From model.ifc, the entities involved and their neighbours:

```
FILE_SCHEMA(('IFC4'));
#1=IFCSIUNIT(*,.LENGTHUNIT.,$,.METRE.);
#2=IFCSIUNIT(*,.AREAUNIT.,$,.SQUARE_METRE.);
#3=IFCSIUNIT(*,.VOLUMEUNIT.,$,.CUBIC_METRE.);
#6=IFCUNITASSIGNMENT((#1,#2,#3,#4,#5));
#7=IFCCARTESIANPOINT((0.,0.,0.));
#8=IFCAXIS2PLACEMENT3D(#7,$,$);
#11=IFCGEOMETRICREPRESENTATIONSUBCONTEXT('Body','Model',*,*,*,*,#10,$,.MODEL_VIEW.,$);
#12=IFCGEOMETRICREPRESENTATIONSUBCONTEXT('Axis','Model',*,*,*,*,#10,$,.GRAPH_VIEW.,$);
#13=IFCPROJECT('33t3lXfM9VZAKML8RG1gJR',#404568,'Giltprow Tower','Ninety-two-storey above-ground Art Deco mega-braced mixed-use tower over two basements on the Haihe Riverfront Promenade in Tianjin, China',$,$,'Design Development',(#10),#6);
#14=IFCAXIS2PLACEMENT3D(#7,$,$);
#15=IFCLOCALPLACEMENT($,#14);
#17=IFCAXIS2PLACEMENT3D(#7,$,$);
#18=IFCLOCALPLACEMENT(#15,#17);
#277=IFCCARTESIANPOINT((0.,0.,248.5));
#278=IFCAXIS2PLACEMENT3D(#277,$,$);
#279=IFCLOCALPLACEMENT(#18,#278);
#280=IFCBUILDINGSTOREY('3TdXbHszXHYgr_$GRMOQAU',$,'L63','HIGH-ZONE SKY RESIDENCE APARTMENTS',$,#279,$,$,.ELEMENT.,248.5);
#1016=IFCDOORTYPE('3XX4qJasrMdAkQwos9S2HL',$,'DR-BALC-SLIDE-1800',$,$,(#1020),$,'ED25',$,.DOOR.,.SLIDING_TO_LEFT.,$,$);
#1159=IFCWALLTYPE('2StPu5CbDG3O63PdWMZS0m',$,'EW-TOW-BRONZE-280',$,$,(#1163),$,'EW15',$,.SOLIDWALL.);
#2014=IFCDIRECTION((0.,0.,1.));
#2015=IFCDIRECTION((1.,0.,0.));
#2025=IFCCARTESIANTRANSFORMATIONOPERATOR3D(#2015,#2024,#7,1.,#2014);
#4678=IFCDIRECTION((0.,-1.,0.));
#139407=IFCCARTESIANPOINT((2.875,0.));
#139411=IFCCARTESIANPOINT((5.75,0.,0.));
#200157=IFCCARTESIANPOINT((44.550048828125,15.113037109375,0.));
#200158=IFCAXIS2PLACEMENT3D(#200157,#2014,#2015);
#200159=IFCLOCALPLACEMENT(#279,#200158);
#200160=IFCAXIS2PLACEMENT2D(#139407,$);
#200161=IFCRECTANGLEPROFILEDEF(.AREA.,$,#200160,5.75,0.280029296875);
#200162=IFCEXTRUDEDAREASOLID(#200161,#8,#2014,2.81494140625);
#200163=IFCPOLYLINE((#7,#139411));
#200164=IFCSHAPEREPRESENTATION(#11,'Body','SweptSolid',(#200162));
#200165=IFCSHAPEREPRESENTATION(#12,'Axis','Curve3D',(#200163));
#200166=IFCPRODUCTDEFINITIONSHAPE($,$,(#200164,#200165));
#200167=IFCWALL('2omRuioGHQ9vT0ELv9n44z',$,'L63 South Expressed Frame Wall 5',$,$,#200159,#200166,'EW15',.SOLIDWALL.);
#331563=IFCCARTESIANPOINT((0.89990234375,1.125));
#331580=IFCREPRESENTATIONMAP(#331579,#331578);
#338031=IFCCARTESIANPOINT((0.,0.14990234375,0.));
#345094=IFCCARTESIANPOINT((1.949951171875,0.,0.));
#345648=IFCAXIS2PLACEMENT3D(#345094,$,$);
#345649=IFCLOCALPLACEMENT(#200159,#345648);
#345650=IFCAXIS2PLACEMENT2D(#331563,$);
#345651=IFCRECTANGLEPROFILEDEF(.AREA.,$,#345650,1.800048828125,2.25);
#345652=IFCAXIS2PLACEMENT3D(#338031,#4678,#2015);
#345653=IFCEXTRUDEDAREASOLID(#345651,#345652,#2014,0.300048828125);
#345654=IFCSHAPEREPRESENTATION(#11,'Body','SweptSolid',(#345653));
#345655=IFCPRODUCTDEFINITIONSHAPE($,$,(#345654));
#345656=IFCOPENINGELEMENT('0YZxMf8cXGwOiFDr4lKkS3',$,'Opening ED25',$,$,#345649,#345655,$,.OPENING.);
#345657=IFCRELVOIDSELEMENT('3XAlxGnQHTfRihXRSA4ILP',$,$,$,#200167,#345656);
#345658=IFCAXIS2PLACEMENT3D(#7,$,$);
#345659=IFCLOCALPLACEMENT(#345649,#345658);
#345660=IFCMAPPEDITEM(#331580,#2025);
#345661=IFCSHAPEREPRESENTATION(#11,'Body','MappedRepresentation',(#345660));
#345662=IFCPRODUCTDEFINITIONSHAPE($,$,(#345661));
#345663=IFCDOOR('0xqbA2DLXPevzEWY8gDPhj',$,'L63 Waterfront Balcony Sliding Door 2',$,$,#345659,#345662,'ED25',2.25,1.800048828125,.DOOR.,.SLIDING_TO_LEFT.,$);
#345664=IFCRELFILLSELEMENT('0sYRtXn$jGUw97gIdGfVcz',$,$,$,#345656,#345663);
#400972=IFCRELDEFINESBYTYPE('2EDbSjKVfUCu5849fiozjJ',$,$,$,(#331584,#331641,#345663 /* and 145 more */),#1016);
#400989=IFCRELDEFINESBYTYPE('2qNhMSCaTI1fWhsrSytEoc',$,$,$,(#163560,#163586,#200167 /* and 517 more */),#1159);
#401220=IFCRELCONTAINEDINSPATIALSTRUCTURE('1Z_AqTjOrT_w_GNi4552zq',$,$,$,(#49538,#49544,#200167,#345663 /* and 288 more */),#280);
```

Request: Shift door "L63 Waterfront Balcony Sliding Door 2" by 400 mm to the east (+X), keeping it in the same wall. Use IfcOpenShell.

```python
import ifcopenshell
import ifcopenshell.api.geometry
import ifcopenshell.util.placement

model = ifcopenshell.open("model.ifc")

door = model.by_guid("0xqbA2DLXPevzEWY8gDPhj")
opening = door.FillsVoids[0].RelatingOpeningElement
wall = opening.VoidsElements[0].RelatingBuildingElement

wall_matrix = ifcopenshell.util.placement.get_local_placement(wall.ObjectPlacement)
shift = wall_matrix[:3, 0] * 0.4
before = ifcopenshell.util.placement.get_local_placement(door.ObjectPlacement)[:3, 3].copy()

# The door is placed relative to its opening, so it follows when the opening moves.
matrix = ifcopenshell.util.placement.get_local_placement(opening.ObjectPlacement)
matrix[:3, 3] += shift
ifcopenshell.api.geometry.edit_object_placement(
    model, product=opening, matrix=matrix, is_si=False, should_transform_children=True
)

after = ifcopenshell.util.placement.get_local_placement(door.ObjectPlacement)[:3, 3]
print("door moved by", (after - before).round(3) + 0.0)

model.write("model_edited.ifc")
```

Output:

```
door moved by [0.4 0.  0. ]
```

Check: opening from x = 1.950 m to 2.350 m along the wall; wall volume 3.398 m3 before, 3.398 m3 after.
